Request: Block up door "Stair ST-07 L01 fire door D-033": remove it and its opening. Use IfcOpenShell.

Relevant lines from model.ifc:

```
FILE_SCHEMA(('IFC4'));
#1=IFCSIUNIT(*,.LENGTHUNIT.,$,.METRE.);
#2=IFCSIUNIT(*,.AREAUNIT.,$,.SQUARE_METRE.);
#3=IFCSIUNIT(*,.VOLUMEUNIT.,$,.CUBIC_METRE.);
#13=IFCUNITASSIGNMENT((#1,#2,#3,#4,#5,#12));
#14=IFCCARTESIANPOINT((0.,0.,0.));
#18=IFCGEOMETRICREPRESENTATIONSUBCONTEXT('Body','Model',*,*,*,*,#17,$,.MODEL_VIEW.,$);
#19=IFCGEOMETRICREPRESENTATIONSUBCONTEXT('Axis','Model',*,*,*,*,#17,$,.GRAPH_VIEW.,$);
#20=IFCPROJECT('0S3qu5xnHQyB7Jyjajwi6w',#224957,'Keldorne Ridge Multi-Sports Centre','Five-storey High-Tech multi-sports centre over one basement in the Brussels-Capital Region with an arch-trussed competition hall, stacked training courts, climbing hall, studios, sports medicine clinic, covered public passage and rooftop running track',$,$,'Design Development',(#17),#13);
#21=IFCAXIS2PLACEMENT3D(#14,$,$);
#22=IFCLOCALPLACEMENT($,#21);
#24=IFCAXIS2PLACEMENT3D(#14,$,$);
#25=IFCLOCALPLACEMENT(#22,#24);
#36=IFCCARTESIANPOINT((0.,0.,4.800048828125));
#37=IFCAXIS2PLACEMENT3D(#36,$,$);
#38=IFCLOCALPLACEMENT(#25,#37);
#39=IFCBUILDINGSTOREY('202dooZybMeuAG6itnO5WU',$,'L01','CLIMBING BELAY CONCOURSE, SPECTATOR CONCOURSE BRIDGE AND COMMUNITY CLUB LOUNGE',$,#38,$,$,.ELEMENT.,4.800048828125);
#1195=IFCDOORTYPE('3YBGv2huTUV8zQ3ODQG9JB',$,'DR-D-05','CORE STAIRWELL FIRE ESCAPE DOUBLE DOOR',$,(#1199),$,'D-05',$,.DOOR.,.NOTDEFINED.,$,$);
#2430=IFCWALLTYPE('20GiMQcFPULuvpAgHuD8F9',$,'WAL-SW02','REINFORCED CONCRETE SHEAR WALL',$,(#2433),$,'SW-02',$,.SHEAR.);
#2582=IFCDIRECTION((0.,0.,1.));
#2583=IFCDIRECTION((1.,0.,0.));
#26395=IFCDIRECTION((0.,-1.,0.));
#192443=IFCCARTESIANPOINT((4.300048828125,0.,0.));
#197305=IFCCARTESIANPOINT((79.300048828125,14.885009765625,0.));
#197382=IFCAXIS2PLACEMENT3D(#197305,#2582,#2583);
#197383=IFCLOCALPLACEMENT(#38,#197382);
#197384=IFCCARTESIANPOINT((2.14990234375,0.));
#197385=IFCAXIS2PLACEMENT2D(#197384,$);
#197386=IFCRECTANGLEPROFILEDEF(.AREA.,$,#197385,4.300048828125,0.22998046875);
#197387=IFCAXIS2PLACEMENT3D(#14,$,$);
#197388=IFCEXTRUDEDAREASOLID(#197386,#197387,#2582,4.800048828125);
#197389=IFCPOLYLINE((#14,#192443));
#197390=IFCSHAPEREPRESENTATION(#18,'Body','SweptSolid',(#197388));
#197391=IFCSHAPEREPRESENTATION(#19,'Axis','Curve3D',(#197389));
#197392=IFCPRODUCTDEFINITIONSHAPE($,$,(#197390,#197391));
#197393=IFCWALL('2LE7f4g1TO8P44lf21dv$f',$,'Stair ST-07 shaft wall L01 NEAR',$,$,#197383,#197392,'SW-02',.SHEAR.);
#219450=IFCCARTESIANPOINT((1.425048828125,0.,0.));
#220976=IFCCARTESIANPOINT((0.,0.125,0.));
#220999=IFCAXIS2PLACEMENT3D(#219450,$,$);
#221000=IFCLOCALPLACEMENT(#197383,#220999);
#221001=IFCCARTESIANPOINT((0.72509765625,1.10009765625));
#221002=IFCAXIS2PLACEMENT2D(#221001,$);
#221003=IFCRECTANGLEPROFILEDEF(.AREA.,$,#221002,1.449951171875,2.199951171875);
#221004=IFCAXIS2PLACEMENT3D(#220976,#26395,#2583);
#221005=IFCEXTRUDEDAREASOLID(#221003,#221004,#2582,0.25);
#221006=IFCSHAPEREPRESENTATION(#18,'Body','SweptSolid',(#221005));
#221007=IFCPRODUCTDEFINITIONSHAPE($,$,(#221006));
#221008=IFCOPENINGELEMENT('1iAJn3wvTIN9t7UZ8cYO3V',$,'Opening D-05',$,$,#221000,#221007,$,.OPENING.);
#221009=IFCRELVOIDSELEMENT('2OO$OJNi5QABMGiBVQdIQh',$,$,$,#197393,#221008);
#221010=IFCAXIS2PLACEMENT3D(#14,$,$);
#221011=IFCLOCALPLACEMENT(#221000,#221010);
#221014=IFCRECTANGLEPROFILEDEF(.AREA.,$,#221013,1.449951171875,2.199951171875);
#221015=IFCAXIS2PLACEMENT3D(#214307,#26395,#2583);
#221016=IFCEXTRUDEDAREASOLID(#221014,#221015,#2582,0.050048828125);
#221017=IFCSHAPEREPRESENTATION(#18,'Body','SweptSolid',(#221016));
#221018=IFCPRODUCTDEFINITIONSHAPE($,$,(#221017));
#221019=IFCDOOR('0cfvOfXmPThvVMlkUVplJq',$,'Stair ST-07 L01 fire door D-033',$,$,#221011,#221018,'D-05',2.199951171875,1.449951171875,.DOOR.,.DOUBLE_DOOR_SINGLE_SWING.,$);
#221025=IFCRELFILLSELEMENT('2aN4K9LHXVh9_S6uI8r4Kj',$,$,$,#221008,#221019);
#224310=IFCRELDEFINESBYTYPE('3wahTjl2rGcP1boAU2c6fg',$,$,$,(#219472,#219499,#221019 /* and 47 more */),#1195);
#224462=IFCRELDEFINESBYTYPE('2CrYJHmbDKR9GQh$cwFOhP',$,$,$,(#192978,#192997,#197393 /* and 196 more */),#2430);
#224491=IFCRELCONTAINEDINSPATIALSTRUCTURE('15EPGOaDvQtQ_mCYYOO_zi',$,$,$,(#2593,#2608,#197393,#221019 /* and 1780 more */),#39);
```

```python
import ifcopenshell
import ifcopenshell.api.feature
import ifcopenshell.api.root
import ifcopenshell.geom
import ifcopenshell.util.shape

model = ifcopenshell.open("model.ifc")
settings = ifcopenshell.geom.settings()


def volume(element):
    """Net volume in cubic metres, openings subtracted."""
    shape = ifcopenshell.geom.create_shape(settings, element)
    return ifcopenshell.util.shape.get_volume(shape.geometry)


door = model.by_guid("0cfvOfXmPThvVMlkUVplJq")
opening = door.FillsVoids[0].RelatingOpeningElement
wall = opening.VoidsElements[0].RelatingBuildingElement
before = volume(wall)

ifcopenshell.api.root.remove_product(model, product=door)
ifcopenshell.api.feature.remove_feature(model, feature=opening)

after = volume(wall)

print(f"wall volume {before:.3f} -> {after:.3f} m3")

model.write("model_edited.ifc")
```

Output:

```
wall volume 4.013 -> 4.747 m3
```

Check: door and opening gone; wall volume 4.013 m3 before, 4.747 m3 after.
